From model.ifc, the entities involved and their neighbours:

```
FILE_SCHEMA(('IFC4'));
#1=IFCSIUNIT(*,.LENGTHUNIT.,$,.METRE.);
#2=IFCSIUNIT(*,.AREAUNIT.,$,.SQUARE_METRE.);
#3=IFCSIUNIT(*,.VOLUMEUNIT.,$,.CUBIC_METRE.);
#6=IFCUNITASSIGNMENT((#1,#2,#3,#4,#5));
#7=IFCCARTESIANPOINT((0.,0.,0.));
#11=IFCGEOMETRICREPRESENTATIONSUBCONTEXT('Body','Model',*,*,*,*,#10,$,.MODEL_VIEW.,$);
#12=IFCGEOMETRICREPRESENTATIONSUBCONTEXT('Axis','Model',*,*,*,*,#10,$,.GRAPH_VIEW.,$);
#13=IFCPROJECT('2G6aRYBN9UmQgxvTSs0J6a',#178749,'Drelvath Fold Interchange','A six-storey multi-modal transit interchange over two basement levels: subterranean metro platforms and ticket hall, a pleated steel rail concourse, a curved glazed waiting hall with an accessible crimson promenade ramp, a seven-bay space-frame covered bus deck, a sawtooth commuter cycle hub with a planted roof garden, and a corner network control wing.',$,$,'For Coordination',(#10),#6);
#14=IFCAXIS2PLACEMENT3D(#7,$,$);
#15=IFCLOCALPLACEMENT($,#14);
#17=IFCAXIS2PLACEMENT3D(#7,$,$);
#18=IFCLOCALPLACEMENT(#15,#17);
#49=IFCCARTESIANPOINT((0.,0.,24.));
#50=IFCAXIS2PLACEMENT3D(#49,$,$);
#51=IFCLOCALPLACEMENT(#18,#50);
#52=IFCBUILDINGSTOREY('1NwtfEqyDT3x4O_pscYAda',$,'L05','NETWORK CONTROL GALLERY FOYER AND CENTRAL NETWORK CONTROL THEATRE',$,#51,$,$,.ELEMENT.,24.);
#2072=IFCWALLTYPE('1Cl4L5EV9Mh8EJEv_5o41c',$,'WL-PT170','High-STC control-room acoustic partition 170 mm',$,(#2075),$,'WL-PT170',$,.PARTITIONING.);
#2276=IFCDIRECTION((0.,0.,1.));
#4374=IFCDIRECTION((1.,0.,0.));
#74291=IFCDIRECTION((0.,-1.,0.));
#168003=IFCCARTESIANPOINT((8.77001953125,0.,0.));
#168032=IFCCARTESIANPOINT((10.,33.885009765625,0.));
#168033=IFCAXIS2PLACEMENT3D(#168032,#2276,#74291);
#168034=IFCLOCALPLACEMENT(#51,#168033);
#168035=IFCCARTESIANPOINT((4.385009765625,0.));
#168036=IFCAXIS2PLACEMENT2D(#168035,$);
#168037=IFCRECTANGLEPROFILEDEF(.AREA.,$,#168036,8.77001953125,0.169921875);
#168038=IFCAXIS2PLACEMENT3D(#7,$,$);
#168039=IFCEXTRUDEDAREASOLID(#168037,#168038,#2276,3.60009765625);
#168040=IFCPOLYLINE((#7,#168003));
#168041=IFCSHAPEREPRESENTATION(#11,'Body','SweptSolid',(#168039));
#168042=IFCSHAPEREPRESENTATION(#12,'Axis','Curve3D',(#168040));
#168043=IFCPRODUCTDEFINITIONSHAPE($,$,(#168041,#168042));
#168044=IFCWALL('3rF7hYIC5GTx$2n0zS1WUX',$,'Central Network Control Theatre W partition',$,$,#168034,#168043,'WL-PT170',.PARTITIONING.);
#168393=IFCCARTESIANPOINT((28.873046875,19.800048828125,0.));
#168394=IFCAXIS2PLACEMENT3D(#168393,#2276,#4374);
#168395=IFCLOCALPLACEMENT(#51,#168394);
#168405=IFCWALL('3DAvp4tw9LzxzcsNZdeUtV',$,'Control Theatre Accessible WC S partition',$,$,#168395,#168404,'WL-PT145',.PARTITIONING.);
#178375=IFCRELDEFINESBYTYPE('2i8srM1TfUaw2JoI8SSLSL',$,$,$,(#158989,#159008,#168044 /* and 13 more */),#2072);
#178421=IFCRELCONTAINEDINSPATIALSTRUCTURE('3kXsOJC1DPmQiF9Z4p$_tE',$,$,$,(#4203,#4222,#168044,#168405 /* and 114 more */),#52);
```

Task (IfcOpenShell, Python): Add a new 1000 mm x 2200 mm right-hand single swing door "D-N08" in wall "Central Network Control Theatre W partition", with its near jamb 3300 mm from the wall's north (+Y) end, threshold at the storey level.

```python
import numpy as np
import ifcopenshell
import ifcopenshell.api.feature
import ifcopenshell.api.geometry
import ifcopenshell.api.root
import ifcopenshell.api.spatial
import ifcopenshell.geom
import ifcopenshell.util.element
import ifcopenshell.util.placement
import ifcopenshell.util.representation
import ifcopenshell.util.shape
import ifcopenshell.util.unit

model = ifcopenshell.open("model.ifc")
unit_scale = ifcopenshell.util.unit.calculate_unit_scale(model)
settings = ifcopenshell.geom.settings()


def volume(element):
    """Net volume in cubic metres, openings subtracted."""
    shape = ifcopenshell.geom.create_shape(settings, element)
    return ifcopenshell.util.shape.get_volume(shape.geometry)


wall = model.by_id(168044)
storey = ifcopenshell.util.element.get_container(wall, ifc_class="IfcBuildingStorey")
context = ifcopenshell.util.representation.get_context(model, "Model", "Body", "MODEL_VIEW")
before = volume(wall)

width, height, from_end, sill = 1, 2.2, 3.3, 0.0  # metres

# The wall runs along its own X axis, and the end named is its -X end.
wall_shape = ifcopenshell.geom.create_shape(settings, wall)
x, y, z = ifcopenshell.util.shape.get_vertices(wall_shape.geometry).T
start = x.min() + from_end
face, thickness = float(y.min()), float(y.max() - y.min())
wall_matrix = ifcopenshell.util.placement.get_local_placement(wall.ObjectPlacement)
level = ifcopenshell.util.placement.get_local_placement(storey.ObjectPlacement)[2, 3]


def in_wall(x, y):
    """Placement at x, y metres in the wall's axes, at sill height."""
    matrix = wall_matrix.copy()
    matrix[:, 3] = wall_matrix @ np.array([x / unit_scale, y / unit_scale, 0.0, 1.0])
    matrix[2, 3] = level + sill / unit_scale
    return matrix


# Opening: a box that overshoots both wall faces by 50 mm.
opening = ifcopenshell.api.root.create_entity(model, ifc_class="IfcOpeningElement", predefined_type="OPENING")
box = ifcopenshell.api.geometry.add_wall_representation(
    model, context=context, length=width, height=height, thickness=thickness + 0.1
)
ifcopenshell.api.geometry.assign_representation(model, product=opening, representation=box)
ifcopenshell.api.geometry.edit_object_placement(model, product=opening, matrix=in_wall(start, face - 0.05), is_si=False)
ifcopenshell.api.feature.add_feature(model, feature=opening, element=wall)

door = ifcopenshell.api.root.create_entity(model, ifc_class="IfcDoor", name="D-N08", predefined_type="DOOR")
door.OverallWidth, door.OverallHeight = width / unit_scale, height / unit_scale
door.OperationType = "SINGLE_SWING_RIGHT"
body = ifcopenshell.api.geometry.add_door_representation(
    model,
    context=context,
    overall_width=door.OverallWidth,
    overall_height=door.OverallHeight,
    operation_type="SINGLE_SWING_RIGHT",
    lining_properties={"LiningDepth": thickness / unit_scale, "ThresholdDepth": thickness / unit_scale},
)
ifcopenshell.api.geometry.assign_representation(model, product=door, representation=body)
ifcopenshell.api.spatial.assign_container(model, products=[door], relating_structure=storey)
ifcopenshell.api.feature.add_filling(model, opening=opening, element=door)

# The lining spans the wall, so the door starts at the wall face.
ifcopenshell.api.geometry.edit_object_placement(model, product=door, matrix=in_wall(start, face), is_si=False)

after = volume(wall)

print(f"wall volume {before:.3f} -> {after:.3f} m3")

model.write("model-out.ifc")
```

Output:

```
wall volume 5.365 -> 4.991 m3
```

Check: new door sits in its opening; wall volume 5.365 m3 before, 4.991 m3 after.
